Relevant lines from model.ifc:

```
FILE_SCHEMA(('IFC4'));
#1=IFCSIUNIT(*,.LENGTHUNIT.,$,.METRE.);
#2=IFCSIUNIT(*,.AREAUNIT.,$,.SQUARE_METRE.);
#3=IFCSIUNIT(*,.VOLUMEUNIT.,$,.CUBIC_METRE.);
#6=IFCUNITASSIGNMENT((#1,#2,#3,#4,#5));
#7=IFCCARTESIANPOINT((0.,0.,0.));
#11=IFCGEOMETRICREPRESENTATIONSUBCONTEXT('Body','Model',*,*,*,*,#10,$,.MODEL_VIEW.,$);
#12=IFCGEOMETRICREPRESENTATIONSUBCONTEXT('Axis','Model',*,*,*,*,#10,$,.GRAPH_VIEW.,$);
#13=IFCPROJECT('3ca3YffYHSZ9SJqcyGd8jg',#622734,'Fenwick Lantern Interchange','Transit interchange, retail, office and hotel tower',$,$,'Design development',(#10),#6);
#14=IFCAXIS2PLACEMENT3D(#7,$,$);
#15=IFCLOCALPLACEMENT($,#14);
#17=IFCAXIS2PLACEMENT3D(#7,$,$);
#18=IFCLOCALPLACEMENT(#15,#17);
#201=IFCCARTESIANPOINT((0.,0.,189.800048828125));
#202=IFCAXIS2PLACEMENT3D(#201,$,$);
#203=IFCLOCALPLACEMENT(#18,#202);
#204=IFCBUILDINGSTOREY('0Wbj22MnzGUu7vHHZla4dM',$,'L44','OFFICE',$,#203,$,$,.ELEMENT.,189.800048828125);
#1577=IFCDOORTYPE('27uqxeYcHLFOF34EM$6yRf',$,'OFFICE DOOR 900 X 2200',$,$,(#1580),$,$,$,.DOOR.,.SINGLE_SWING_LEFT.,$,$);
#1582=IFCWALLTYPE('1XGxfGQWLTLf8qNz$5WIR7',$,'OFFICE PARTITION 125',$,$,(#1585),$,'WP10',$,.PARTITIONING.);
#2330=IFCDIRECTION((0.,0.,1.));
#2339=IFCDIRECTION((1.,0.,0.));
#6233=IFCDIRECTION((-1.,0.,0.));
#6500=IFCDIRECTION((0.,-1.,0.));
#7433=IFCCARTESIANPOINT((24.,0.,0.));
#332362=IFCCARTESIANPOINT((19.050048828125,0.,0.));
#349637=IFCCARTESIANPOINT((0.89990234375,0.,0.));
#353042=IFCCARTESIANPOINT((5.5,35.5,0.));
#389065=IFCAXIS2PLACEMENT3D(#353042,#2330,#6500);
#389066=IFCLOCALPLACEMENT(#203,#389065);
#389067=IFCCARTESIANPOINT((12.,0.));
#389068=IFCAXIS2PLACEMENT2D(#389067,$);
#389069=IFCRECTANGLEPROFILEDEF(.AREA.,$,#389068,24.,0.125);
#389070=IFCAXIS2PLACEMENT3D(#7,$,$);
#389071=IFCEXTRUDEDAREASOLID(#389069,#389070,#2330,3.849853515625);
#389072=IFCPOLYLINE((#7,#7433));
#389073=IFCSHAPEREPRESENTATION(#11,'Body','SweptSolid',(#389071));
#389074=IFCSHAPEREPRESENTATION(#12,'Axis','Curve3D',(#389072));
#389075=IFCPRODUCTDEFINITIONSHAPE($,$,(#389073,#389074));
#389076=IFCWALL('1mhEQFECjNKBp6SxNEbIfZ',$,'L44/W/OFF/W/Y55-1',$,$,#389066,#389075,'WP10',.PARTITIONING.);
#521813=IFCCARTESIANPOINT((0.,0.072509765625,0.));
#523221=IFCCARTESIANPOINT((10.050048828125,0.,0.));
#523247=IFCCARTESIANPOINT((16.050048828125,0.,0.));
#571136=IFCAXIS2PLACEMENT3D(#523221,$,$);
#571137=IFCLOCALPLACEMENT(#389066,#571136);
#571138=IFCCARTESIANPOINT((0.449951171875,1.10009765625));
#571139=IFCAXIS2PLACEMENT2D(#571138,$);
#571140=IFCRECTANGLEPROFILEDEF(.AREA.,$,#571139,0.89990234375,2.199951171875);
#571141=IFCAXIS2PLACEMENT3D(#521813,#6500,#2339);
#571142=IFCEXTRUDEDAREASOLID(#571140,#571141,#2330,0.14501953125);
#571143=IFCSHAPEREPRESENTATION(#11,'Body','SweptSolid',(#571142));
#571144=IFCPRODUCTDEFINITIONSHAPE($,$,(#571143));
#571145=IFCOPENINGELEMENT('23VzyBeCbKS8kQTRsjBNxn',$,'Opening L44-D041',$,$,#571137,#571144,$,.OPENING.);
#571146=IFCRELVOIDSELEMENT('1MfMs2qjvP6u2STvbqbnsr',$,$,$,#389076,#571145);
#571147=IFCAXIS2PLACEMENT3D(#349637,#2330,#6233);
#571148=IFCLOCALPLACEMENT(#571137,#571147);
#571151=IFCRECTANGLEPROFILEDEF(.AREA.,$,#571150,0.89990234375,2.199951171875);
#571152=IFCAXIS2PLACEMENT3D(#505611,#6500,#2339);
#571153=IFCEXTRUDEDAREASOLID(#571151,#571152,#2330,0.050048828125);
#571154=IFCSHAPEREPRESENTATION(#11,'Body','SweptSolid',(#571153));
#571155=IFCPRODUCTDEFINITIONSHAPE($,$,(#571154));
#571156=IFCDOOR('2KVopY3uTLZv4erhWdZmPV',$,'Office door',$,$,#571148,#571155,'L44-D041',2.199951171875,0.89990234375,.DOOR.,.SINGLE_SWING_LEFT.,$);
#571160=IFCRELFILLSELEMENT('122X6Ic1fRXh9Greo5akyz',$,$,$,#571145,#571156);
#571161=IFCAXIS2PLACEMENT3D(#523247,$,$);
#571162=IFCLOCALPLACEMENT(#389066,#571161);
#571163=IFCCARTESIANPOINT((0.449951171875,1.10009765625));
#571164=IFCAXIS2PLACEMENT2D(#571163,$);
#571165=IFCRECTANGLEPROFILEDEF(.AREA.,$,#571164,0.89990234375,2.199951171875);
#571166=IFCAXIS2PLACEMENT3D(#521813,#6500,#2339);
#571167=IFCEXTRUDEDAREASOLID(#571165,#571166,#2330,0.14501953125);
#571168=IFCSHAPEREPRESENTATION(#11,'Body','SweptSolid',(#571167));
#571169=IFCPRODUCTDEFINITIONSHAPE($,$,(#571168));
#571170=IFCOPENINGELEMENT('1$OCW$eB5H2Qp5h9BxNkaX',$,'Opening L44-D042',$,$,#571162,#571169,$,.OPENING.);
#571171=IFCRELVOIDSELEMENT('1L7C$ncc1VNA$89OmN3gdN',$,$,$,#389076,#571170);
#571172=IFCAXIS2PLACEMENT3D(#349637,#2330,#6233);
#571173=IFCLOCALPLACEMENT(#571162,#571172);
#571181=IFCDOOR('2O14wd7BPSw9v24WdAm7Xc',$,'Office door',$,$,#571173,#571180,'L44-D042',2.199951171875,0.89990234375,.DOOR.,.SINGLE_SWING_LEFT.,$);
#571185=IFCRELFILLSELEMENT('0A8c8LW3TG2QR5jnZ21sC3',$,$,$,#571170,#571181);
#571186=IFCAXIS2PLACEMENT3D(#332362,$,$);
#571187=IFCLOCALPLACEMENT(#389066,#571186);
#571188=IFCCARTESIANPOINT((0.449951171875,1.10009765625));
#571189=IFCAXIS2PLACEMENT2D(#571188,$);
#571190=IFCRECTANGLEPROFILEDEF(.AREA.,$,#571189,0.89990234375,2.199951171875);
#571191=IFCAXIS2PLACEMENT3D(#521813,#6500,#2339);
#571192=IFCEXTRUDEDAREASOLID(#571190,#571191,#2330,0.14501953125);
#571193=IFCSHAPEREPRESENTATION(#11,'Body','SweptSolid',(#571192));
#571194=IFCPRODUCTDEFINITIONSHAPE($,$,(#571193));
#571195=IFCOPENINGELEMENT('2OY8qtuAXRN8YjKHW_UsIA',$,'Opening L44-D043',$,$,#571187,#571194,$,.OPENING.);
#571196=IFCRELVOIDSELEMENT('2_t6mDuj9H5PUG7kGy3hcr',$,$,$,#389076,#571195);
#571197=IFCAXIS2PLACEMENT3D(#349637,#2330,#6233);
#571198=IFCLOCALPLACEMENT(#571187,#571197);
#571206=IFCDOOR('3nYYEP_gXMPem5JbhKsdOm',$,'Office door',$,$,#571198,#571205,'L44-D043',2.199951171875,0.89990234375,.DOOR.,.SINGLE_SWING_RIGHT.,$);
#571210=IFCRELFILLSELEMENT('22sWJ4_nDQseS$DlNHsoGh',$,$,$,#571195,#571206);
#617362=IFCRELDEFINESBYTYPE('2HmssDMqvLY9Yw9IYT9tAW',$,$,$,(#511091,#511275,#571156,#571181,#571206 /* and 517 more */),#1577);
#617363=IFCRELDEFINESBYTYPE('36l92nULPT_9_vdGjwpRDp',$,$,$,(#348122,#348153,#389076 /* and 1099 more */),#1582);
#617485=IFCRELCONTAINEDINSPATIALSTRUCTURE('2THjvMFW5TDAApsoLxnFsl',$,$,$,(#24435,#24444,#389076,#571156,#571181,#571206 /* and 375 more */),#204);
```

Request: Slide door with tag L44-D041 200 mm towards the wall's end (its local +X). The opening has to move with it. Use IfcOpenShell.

```python
import ifcopenshell
import ifcopenshell.api.geometry
import ifcopenshell.util.placement
import ifcopenshell.util.unit

model = ifcopenshell.open("model.ifc")
unit_scale = ifcopenshell.util.unit.calculate_unit_scale(model)

door = model.by_guid("2KVopY3uTLZv4erhWdZmPV")
opening = door.FillsVoids[0].RelatingOpeningElement
wall = opening.VoidsElements[0].RelatingBuildingElement

wall_matrix = ifcopenshell.util.placement.get_local_placement(wall.ObjectPlacement)
shift = wall_matrix[:3, 0] * 0.2 / unit_scale
before = ifcopenshell.util.placement.get_local_placement(door.ObjectPlacement)[:3, 3].copy()

# The door is placed relative to its opening, so it follows when the opening moves.
matrix = ifcopenshell.util.placement.get_local_placement(opening.ObjectPlacement)
matrix[:3, 3] += shift
ifcopenshell.api.geometry.edit_object_placement(
    model, product=opening, matrix=matrix, is_si=False, should_transform_children=True
)

after = ifcopenshell.util.placement.get_local_placement(door.ObjectPlacement)[:3, 3]
print("door moved by", (after - before).round(3) + 0.0)

model.write("model_rev.ifc")
```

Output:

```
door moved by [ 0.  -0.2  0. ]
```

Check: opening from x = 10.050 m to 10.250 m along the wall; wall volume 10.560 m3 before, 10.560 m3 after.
